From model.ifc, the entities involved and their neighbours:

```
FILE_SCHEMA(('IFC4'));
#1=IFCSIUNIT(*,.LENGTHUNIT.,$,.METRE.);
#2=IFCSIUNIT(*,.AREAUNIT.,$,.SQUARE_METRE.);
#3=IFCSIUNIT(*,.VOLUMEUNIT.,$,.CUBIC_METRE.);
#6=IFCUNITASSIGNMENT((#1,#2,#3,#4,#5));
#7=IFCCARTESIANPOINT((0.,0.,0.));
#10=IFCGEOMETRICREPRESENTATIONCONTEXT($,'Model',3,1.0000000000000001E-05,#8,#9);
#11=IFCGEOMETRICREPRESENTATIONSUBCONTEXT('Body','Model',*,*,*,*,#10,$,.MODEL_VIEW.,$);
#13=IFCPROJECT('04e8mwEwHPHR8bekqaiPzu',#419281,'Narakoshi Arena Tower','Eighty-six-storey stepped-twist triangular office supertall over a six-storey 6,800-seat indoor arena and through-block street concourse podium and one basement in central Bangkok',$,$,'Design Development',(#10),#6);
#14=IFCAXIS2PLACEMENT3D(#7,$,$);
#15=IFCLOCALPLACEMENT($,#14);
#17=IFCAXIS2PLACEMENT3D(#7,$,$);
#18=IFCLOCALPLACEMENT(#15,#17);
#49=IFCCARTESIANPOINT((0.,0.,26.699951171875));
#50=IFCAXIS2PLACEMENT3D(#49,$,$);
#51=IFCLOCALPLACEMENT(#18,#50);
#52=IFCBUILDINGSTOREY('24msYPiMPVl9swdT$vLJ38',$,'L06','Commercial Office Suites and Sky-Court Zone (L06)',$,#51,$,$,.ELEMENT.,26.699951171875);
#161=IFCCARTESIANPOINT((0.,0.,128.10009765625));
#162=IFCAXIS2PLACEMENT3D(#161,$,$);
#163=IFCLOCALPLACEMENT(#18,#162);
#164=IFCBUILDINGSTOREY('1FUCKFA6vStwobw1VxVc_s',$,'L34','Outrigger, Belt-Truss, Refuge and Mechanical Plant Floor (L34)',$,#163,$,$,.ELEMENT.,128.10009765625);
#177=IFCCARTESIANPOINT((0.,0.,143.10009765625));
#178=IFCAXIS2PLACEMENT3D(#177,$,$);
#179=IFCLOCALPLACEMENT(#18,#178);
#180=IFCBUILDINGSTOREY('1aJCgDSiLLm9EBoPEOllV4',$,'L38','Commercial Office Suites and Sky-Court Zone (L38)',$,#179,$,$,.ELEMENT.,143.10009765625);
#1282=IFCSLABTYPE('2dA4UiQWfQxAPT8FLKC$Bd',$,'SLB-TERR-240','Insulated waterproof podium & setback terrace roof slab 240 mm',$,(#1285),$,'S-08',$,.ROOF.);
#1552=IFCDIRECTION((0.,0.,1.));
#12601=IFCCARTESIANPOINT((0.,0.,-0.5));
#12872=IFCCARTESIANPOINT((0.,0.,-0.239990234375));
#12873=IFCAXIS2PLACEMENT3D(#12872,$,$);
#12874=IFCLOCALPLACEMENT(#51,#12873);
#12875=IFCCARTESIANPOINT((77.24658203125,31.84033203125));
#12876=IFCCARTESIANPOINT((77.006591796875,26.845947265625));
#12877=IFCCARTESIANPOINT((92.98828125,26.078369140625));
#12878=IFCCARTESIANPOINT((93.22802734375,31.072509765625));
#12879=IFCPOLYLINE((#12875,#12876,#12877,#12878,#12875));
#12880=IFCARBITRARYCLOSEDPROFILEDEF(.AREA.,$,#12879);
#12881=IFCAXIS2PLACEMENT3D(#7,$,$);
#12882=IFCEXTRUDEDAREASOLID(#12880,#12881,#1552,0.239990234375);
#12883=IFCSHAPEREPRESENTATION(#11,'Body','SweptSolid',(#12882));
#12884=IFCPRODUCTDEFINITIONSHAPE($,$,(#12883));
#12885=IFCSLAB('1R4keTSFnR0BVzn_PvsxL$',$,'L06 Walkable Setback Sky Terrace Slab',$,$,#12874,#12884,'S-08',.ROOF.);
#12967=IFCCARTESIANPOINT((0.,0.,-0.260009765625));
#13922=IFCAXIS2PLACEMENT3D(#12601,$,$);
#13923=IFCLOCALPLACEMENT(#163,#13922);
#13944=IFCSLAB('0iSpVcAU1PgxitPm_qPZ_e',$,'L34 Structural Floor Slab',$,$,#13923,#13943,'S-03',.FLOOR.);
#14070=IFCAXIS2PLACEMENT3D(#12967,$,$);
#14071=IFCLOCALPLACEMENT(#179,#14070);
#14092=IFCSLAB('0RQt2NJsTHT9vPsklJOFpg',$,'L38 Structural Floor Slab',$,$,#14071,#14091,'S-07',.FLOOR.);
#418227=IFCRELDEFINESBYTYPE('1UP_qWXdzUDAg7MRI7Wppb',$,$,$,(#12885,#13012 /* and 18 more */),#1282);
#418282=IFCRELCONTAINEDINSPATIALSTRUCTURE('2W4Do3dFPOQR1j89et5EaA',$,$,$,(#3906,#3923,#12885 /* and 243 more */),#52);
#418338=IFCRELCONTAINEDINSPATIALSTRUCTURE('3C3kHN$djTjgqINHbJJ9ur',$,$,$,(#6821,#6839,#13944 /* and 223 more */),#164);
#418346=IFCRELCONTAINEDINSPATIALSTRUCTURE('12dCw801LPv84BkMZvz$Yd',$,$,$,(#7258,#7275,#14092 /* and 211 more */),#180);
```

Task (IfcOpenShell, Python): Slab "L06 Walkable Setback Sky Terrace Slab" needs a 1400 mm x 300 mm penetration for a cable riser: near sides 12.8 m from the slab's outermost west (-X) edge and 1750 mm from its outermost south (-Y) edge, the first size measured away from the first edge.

```python
import numpy as np
import ifcopenshell
import ifcopenshell.api.feature
import ifcopenshell.api.geometry
import ifcopenshell.api.root
import ifcopenshell.geom
import ifcopenshell.util.placement
import ifcopenshell.util.representation
import ifcopenshell.util.shape
import ifcopenshell.util.unit

model = ifcopenshell.open("model.ifc")
unit_scale = ifcopenshell.util.unit.calculate_unit_scale(model)
settings = ifcopenshell.geom.settings()


def volume(element):
    """Net volume in cubic metres, openings subtracted."""
    shape = ifcopenshell.geom.create_shape(settings, element)
    return ifcopenshell.util.shape.get_volume(shape.geometry)


slab = model.by_guid("1R4keTSFnR0BVzn_PvsxL$")
before = volume(slab)

# Extent in the slab's own axes, in metres. The edges named are its -X and -Y sides.
slab_shape = ifcopenshell.geom.create_shape(settings, slab)
vertices = ifcopenshell.util.shape.get_vertices(slab_shape.geometry)
x_min, y_min, bottom = vertices.min(axis=0)
top = vertices[:, 2].max()

opening = ifcopenshell.api.root.create_entity(model, ifc_class="IfcOpeningElement", name="Cable riser opening", predefined_type="OPENING")
context = ifcopenshell.util.representation.get_context(model, "Model", "Body", "MODEL_VIEW")
width, depth = 1.4, 0.3
outline = [(0.0, 0.0), (width, 0.0), (width, depth), (0.0, depth), (0.0, 0.0)]
# Overshoot both faces by 50 mm so the cut is clean.
shape = ifcopenshell.api.geometry.add_slab_representation(
    model, context=context, depth=top - bottom + 0.1, polyline=outline
)
ifcopenshell.api.geometry.assign_representation(model, product=opening, representation=shape)

matrix = ifcopenshell.util.placement.get_local_placement(slab.ObjectPlacement)
matrix[:, 3] = matrix @ np.append(np.array([x_min + 12.8, y_min + 1.75, bottom - 0.05]) / unit_scale, 1.0)
ifcopenshell.api.geometry.edit_object_placement(model, product=opening, matrix=matrix, is_si=False)
ifcopenshell.api.feature.add_feature(model, feature=opening, element=slab)

after = volume(slab)

print(f"slab volume {before:.3f} -> {after:.3f} m3")

model.write("model_rev.ifc")
```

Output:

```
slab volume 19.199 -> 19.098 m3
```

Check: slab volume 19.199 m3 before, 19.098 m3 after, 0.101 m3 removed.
